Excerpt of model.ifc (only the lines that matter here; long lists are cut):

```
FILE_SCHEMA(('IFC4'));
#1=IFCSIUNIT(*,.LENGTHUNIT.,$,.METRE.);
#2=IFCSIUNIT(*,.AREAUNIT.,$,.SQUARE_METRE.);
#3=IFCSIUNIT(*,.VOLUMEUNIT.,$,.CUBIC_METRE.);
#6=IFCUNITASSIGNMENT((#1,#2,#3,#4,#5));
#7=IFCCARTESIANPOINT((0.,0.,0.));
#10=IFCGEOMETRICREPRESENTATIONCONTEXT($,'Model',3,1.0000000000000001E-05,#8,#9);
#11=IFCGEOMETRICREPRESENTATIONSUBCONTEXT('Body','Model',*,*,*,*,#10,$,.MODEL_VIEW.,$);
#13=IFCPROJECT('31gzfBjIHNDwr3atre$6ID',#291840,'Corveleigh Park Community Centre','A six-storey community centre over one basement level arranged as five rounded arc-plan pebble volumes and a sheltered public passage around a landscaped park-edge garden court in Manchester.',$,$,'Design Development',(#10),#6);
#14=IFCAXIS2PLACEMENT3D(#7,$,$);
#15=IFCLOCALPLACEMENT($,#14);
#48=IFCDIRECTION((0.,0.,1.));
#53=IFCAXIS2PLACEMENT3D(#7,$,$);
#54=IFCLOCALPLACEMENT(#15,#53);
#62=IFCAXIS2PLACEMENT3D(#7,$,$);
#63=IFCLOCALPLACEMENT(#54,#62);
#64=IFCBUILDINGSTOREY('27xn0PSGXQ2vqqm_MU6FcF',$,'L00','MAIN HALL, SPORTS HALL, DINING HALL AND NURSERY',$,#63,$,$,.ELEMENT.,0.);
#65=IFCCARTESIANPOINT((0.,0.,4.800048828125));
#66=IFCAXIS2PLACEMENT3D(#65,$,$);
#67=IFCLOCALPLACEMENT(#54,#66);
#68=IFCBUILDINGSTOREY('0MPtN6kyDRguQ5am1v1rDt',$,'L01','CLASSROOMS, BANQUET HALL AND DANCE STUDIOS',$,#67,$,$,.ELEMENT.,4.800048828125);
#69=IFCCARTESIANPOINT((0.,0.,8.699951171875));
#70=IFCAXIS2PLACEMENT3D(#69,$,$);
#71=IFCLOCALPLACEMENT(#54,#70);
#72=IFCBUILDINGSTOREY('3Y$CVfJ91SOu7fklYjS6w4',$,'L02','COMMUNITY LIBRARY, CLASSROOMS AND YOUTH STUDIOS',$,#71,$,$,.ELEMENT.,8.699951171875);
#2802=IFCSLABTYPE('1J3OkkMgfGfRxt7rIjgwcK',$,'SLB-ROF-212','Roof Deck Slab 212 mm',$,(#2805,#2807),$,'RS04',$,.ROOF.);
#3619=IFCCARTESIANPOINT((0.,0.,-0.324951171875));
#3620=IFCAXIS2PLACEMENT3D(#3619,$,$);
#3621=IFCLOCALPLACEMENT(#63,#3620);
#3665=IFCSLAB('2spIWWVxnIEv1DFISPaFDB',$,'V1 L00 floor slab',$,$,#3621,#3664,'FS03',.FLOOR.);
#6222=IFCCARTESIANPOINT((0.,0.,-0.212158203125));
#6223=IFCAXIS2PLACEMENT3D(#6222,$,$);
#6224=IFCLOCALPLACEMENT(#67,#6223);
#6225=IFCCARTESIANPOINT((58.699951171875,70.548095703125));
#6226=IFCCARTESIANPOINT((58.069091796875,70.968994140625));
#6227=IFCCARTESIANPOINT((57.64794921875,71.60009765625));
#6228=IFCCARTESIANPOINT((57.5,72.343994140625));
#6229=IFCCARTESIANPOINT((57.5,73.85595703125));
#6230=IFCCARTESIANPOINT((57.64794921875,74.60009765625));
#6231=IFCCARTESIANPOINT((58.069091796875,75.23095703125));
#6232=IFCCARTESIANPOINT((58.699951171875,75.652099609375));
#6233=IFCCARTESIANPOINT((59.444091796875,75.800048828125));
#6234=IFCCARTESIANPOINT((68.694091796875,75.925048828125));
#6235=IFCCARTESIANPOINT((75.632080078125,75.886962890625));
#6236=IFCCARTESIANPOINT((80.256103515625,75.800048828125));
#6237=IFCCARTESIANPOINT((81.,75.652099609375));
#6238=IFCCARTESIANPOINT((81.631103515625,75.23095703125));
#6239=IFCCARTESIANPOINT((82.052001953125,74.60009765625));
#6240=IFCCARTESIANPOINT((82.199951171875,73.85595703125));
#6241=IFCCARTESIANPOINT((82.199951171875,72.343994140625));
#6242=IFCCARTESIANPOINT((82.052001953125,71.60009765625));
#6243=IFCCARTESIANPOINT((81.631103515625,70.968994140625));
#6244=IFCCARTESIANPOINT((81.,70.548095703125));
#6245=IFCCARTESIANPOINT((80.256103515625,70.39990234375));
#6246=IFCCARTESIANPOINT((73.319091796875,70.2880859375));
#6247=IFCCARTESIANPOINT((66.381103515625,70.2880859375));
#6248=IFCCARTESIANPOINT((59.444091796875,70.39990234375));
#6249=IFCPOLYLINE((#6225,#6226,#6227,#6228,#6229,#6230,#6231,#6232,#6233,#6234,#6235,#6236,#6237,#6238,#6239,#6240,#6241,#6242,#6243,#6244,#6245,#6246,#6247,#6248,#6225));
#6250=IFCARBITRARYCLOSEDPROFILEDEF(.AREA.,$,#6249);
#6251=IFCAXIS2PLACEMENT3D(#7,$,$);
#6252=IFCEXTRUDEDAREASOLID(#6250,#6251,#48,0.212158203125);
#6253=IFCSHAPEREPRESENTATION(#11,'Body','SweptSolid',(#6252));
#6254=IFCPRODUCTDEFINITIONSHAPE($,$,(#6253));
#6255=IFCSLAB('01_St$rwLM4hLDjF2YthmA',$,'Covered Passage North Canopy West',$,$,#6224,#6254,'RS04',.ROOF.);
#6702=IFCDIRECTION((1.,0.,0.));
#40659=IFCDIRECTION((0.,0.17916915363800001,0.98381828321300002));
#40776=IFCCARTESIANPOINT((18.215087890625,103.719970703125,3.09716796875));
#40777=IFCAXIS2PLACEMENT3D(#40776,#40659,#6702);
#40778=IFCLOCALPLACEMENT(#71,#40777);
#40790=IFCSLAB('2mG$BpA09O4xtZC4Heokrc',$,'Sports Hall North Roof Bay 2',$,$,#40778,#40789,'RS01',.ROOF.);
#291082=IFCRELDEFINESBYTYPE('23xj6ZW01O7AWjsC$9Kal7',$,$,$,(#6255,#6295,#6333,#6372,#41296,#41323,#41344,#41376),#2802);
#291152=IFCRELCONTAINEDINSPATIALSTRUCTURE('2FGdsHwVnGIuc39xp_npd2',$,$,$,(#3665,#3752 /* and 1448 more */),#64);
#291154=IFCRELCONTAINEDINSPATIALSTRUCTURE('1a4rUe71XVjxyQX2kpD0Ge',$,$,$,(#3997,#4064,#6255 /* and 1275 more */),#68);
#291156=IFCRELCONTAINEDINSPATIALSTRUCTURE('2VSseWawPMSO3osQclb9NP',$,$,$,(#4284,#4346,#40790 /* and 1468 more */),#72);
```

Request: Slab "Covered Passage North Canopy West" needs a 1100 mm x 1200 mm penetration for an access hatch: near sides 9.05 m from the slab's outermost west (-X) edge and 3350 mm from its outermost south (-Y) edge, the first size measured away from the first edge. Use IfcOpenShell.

```python
import numpy as np
import ifcopenshell
import ifcopenshell.api.feature
import ifcopenshell.api.geometry
import ifcopenshell.api.root
import ifcopenshell.geom
import ifcopenshell.util.placement
import ifcopenshell.util.representation
import ifcopenshell.util.shape
import ifcopenshell.util.unit

model = ifcopenshell.open("model.ifc")
unit_scale = ifcopenshell.util.unit.calculate_unit_scale(model)
settings = ifcopenshell.geom.settings()


def volume(element):
    """Net volume in cubic metres, openings subtracted."""
    shape = ifcopenshell.geom.create_shape(settings, element)
    return ifcopenshell.util.shape.get_volume(shape.geometry)


slab = model.by_id(6255)
before = volume(slab)

# Extent in the slab's own axes, in metres. The edges named are its -X and -Y sides.
slab_shape = ifcopenshell.geom.create_shape(settings, slab)
vertices = ifcopenshell.util.shape.get_vertices(slab_shape.geometry)
x_min, y_min, bottom = vertices.min(axis=0)
top = vertices[:, 2].max()

opening = ifcopenshell.api.root.create_entity(model, ifc_class="IfcOpeningElement", name="Access hatch opening", predefined_type="OPENING")
context = ifcopenshell.util.representation.get_context(model, "Model", "Body", "MODEL_VIEW")
width, depth = 1.1, 1.2
outline = [(0.0, 0.0), (width, 0.0), (width, depth), (0.0, depth), (0.0, 0.0)]
# Overshoot both faces by 50 mm so the cut is clean.
shape = ifcopenshell.api.geometry.add_slab_representation(
    model, context=context, depth=top - bottom + 0.1, polyline=outline
)
ifcopenshell.api.geometry.assign_representation(model, product=opening, representation=shape)

matrix = ifcopenshell.util.placement.get_local_placement(slab.ObjectPlacement)
matrix[:, 3] = matrix @ np.append(np.array([x_min + 9.05, y_min + 3.35, bottom - 0.05]) / unit_scale, 1.0)
ifcopenshell.api.geometry.edit_object_placement(model, product=opening, matrix=matrix, is_si=False)
ifcopenshell.api.feature.add_feature(model, feature=opening, element=slab)

after = volume(slab)

print(f"slab volume {before:.3f} -> {after:.3f} m3")

model.write("model_updated.ifc")
```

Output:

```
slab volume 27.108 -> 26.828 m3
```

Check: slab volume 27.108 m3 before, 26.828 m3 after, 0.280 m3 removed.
